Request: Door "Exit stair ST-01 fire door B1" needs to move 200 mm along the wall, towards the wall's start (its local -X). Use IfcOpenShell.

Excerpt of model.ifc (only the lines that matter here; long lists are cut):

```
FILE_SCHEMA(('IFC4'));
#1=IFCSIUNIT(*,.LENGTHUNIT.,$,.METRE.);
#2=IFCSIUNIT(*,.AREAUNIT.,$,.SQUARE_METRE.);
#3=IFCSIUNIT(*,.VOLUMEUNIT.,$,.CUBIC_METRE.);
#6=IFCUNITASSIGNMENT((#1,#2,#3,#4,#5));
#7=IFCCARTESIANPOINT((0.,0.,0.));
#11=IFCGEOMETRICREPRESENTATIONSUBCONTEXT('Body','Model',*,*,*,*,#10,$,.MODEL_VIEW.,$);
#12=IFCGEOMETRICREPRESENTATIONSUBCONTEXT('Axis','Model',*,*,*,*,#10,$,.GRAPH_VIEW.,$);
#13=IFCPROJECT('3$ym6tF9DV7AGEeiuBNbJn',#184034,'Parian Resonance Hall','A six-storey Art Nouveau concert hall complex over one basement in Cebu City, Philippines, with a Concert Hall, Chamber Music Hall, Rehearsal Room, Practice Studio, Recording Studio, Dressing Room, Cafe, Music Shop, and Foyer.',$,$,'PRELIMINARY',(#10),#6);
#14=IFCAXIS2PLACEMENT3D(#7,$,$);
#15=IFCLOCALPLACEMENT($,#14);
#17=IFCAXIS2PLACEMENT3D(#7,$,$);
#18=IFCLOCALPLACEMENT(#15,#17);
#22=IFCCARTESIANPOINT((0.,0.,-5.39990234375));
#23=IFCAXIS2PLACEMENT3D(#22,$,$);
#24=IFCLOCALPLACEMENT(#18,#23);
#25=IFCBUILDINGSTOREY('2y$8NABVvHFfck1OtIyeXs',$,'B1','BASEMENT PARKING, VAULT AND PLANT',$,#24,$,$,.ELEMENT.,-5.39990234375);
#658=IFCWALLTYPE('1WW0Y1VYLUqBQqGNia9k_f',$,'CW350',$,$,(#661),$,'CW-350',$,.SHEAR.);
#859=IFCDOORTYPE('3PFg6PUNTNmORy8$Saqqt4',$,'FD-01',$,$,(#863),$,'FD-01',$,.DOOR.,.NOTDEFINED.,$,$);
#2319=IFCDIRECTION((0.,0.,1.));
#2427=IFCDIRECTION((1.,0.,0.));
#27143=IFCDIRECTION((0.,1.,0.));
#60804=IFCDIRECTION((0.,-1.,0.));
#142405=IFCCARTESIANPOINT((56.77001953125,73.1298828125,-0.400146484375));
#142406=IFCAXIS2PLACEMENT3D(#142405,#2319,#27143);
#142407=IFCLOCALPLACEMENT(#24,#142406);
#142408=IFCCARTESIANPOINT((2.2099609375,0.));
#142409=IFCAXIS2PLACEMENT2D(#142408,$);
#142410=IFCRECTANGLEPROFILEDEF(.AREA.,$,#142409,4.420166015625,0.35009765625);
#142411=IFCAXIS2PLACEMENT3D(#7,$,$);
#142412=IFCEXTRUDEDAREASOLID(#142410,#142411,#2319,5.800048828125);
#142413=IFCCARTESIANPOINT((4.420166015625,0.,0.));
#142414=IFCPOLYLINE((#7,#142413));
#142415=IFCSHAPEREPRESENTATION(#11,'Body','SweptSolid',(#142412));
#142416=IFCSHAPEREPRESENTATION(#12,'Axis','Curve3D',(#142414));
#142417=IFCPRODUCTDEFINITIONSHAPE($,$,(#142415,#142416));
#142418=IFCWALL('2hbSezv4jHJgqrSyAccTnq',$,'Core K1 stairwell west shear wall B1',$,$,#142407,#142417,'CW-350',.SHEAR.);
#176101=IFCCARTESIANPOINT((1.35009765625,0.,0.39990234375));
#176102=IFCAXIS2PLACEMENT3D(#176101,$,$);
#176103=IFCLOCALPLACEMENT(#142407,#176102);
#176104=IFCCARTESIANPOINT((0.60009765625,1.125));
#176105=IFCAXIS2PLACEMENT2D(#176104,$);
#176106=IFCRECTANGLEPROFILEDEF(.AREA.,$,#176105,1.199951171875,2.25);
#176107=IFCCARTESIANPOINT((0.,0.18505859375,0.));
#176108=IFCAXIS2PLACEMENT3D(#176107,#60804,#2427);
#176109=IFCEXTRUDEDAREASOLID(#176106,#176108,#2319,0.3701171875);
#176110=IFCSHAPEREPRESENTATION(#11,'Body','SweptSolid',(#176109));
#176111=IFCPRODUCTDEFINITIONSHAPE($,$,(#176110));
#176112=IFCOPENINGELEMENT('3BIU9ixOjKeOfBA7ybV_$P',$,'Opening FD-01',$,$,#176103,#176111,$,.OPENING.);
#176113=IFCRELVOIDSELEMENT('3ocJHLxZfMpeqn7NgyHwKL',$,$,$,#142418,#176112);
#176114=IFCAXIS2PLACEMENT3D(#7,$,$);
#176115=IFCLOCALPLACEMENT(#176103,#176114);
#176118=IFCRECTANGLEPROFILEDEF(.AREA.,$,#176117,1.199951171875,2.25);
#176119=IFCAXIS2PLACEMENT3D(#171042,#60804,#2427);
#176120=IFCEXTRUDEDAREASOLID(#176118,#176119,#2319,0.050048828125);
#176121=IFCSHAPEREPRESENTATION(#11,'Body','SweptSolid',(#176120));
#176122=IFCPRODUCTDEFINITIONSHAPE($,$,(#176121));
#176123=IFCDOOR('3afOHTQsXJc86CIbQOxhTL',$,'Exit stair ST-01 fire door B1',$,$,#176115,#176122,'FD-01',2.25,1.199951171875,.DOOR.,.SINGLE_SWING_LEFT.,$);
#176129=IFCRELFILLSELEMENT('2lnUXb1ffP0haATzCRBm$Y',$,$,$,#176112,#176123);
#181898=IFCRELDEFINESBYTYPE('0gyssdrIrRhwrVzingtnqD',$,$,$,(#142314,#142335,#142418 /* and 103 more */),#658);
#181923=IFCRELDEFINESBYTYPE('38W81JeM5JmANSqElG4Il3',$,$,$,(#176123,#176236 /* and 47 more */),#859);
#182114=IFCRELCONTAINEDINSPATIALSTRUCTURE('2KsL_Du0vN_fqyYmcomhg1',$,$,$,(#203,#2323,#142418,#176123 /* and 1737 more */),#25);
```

```python
import ifcopenshell
import ifcopenshell.api.geometry
import ifcopenshell.util.placement

model = ifcopenshell.open("model.ifc")

door = model.by_guid("3afOHTQsXJc86CIbQOxhTL")
opening = door.FillsVoids[0].RelatingOpeningElement
wall = opening.VoidsElements[0].RelatingBuildingElement

wall_matrix = ifcopenshell.util.placement.get_local_placement(wall.ObjectPlacement)
shift = wall_matrix[:3, 0] * -0.2
before = ifcopenshell.util.placement.get_local_placement(door.ObjectPlacement)[:3, 3].copy()

# The door is placed relative to its opening, so it follows when the opening moves.
matrix = ifcopenshell.util.placement.get_local_placement(opening.ObjectPlacement)
matrix[:3, 3] += shift
ifcopenshell.api.geometry.edit_object_placement(
    model, product=opening, matrix=matrix, is_si=False, should_transform_children=True
)

after = ifcopenshell.util.placement.get_local_placement(door.ObjectPlacement)[:3, 3]
print("door moved by", (after - before).round(3) + 0.0)

model.write("model_v2.ifc")
```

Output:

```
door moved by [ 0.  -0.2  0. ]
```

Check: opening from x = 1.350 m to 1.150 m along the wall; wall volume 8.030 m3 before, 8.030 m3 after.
